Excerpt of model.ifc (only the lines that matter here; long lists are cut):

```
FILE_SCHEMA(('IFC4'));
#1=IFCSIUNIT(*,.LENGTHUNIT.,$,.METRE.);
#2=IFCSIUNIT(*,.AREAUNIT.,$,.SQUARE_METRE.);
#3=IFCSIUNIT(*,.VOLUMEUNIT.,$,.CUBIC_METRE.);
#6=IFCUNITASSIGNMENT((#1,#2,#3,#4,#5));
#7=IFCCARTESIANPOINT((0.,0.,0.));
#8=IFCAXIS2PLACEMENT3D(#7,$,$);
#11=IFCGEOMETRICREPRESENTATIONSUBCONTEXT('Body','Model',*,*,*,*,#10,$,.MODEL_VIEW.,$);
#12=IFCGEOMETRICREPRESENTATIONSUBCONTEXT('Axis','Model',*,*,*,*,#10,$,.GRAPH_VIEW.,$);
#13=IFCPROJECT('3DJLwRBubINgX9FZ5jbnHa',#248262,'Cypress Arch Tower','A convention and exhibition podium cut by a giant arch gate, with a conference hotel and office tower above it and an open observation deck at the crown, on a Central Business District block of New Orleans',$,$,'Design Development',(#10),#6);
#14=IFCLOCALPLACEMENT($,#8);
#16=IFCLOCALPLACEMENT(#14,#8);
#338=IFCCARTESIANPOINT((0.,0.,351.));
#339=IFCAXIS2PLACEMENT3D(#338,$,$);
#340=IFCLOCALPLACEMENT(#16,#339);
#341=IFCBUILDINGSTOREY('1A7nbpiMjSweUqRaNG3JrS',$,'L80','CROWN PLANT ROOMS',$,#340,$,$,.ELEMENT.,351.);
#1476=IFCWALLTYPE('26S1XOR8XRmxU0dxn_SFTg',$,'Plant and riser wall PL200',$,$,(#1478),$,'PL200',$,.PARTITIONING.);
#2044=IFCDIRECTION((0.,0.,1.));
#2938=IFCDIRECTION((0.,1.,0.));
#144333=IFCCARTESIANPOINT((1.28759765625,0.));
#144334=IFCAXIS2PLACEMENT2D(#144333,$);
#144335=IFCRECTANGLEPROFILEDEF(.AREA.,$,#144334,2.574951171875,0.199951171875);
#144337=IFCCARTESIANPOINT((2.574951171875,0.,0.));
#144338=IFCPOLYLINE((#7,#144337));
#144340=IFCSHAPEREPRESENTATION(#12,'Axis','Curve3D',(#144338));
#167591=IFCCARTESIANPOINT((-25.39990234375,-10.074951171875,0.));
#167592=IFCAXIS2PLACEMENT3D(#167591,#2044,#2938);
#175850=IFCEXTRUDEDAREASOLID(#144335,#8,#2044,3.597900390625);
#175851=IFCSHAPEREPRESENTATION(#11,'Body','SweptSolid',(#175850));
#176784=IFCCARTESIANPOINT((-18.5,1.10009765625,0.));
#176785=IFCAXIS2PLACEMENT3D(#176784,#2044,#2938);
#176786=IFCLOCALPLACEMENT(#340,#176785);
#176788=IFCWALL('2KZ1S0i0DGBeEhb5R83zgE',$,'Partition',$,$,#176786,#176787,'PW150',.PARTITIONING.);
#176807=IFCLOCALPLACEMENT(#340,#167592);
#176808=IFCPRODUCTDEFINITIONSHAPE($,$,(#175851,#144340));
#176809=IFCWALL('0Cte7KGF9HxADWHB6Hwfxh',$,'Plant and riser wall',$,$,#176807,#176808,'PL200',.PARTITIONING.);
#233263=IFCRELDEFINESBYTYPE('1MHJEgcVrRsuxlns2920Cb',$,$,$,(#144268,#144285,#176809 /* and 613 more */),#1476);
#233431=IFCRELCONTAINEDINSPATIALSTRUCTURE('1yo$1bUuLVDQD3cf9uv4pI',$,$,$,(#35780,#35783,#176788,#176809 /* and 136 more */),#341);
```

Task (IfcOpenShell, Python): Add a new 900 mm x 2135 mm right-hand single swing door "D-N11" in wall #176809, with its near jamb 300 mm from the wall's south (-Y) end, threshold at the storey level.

```python
import numpy as np
import ifcopenshell
import ifcopenshell.api.feature
import ifcopenshell.api.geometry
import ifcopenshell.api.root
import ifcopenshell.api.spatial
import ifcopenshell.geom
import ifcopenshell.util.element
import ifcopenshell.util.placement
import ifcopenshell.util.representation
import ifcopenshell.util.shape
import ifcopenshell.util.unit

model = ifcopenshell.open("model.ifc")
unit_scale = ifcopenshell.util.unit.calculate_unit_scale(model)
settings = ifcopenshell.geom.settings()


def volume(element):
    """Net volume in cubic metres, openings subtracted."""
    shape = ifcopenshell.geom.create_shape(settings, element)
    return ifcopenshell.util.shape.get_volume(shape.geometry)


wall = model.by_guid("0Cte7KGF9HxADWHB6Hwfxh")
storey = ifcopenshell.util.element.get_container(wall, ifc_class="IfcBuildingStorey")
context = ifcopenshell.util.representation.get_context(model, "Model", "Body", "MODEL_VIEW")
before = volume(wall)

width, height, from_end, sill = 0.9, 2.135, 0.3, 0.0  # metres

# The wall runs along its own X axis, and the end named is its -X end.
wall_shape = ifcopenshell.geom.create_shape(settings, wall)
x, y, z = ifcopenshell.util.shape.get_vertices(wall_shape.geometry).T
start = x.min() + from_end
face, thickness = float(y.min()), float(y.max() - y.min())
wall_matrix = ifcopenshell.util.placement.get_local_placement(wall.ObjectPlacement)
level = ifcopenshell.util.placement.get_local_placement(storey.ObjectPlacement)[2, 3]


def in_wall(x, y):
    """Placement at x, y metres in the wall's axes, at sill height."""
    matrix = wall_matrix.copy()
    matrix[:, 3] = wall_matrix @ np.array([x / unit_scale, y / unit_scale, 0.0, 1.0])
    matrix[2, 3] = level + sill / unit_scale
    return matrix


# Opening: a box that overshoots both wall faces by 50 mm.
opening = ifcopenshell.api.root.create_entity(model, ifc_class="IfcOpeningElement", predefined_type="OPENING")
box = ifcopenshell.api.geometry.add_wall_representation(
    model, context=context, length=width, height=height, thickness=thickness + 0.1
)
ifcopenshell.api.geometry.assign_representation(model, product=opening, representation=box)
ifcopenshell.api.geometry.edit_object_placement(model, product=opening, matrix=in_wall(start, face - 0.05), is_si=False)
ifcopenshell.api.feature.add_feature(model, feature=opening, element=wall)

door = ifcopenshell.api.root.create_entity(model, ifc_class="IfcDoor", name="D-N11", predefined_type="DOOR")
door.OverallWidth, door.OverallHeight = width / unit_scale, height / unit_scale
door.OperationType = "SINGLE_SWING_RIGHT"
body = ifcopenshell.api.geometry.add_door_representation(
    model,
    context=context,
    overall_width=door.OverallWidth,
    overall_height=door.OverallHeight,
    operation_type="SINGLE_SWING_RIGHT",
    lining_properties={"LiningDepth": thickness / unit_scale, "ThresholdDepth": thickness / unit_scale},
)
ifcopenshell.api.geometry.assign_representation(model, product=door, representation=body)
ifcopenshell.api.spatial.assign_container(model, products=[door], relating_structure=storey)
ifcopenshell.api.feature.add_filling(model, opening=opening, element=door)

# The lining spans the wall, so the door starts at the wall face.
ifcopenshell.api.geometry.edit_object_placement(model, product=door, matrix=in_wall(start, face), is_si=False)

after = volume(wall)

print(f"wall volume {before:.3f} -> {after:.3f} m3")

model.write("model_updated.ifc")
```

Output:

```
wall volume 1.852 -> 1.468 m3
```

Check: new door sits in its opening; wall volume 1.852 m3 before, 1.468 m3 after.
